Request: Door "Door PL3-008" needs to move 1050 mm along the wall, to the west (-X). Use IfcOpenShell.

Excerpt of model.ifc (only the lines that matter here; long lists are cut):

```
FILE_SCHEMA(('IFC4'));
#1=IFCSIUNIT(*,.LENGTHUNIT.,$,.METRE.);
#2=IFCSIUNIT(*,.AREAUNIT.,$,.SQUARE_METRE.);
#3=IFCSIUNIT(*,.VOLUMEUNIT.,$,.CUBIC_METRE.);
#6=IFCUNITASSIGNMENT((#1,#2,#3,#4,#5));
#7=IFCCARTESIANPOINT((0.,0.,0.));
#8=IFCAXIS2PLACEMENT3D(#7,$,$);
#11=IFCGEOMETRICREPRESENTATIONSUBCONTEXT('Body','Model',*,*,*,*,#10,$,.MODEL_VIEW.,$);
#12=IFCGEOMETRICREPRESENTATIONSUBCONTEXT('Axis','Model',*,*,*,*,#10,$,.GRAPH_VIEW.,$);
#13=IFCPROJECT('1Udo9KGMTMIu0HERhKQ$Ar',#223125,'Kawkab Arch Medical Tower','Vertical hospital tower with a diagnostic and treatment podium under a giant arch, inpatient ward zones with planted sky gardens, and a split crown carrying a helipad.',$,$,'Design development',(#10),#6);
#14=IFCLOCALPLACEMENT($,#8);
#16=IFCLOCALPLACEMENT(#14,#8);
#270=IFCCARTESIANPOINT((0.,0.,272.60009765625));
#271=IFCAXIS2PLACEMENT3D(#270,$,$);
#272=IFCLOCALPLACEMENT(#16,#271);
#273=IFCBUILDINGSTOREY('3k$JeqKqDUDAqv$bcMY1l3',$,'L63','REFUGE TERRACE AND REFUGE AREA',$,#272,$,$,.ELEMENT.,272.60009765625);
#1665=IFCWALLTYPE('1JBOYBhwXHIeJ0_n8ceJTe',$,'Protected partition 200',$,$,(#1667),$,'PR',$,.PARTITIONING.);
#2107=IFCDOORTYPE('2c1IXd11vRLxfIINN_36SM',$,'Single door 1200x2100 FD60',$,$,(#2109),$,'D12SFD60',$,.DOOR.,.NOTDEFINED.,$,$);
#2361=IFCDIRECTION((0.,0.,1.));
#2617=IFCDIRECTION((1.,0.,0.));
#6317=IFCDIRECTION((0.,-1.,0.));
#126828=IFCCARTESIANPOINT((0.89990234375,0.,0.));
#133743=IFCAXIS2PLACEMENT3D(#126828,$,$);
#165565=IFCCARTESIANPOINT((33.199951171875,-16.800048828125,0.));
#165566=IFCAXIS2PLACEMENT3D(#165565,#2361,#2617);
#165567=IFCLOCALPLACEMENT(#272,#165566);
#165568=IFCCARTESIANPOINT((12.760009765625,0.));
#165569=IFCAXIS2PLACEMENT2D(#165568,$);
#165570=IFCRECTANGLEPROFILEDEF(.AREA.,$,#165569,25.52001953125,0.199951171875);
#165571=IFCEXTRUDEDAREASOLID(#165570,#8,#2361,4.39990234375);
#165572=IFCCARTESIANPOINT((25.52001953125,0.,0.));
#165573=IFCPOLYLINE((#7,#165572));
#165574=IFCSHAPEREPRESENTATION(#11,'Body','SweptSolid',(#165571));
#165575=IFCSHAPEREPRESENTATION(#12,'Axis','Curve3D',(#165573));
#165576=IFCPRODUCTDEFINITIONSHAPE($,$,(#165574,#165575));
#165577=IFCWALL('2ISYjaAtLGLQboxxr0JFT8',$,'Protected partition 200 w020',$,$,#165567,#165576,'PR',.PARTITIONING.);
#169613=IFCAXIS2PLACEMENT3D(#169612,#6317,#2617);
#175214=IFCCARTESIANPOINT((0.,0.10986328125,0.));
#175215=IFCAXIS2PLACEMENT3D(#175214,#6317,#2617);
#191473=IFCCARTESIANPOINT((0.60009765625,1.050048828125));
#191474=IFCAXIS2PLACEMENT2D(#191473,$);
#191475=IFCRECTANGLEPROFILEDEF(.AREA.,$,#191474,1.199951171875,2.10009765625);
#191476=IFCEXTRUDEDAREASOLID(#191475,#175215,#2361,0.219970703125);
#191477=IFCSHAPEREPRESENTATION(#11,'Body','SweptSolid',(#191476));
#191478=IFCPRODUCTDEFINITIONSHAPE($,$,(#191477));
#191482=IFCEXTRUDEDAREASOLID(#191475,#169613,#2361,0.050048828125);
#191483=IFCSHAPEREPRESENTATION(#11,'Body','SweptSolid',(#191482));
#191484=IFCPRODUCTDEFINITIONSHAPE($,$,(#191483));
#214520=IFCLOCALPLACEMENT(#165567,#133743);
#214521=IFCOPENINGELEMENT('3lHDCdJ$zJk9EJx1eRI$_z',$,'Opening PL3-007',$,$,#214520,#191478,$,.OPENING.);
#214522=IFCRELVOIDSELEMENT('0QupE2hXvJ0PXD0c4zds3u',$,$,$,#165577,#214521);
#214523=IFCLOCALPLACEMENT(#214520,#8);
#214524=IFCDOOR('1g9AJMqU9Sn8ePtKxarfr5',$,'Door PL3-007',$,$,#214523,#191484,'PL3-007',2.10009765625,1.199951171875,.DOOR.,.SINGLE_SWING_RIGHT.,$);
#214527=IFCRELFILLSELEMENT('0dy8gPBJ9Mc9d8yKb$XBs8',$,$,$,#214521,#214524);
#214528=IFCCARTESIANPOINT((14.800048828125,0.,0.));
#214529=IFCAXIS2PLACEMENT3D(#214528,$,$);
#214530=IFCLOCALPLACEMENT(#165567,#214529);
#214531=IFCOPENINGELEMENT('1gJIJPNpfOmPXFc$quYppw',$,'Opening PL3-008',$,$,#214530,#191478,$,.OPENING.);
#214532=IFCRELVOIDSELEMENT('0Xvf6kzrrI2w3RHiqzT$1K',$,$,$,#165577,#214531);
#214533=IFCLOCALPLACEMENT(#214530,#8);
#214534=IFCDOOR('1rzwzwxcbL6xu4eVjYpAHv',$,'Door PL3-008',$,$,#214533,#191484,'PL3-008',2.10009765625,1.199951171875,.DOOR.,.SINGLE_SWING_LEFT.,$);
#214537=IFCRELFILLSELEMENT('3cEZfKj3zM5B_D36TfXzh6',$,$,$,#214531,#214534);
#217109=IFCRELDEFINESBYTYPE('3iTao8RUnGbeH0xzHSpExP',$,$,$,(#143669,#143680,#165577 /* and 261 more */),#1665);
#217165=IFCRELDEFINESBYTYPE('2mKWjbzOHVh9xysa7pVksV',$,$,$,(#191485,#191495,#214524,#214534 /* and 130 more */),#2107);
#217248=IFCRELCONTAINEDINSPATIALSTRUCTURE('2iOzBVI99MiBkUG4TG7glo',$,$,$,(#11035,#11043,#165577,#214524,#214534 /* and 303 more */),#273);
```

```python
import ifcopenshell
import ifcopenshell.api.geometry
import ifcopenshell.util.placement
import ifcopenshell.util.unit

model = ifcopenshell.open("model.ifc")
unit_scale = ifcopenshell.util.unit.calculate_unit_scale(model)

door = model.by_guid("1rzwzwxcbL6xu4eVjYpAHv")
opening = door.FillsVoids[0].RelatingOpeningElement
wall = opening.VoidsElements[0].RelatingBuildingElement

wall_matrix = ifcopenshell.util.placement.get_local_placement(wall.ObjectPlacement)
shift = wall_matrix[:3, 0] * -1.05 / unit_scale
before = ifcopenshell.util.placement.get_local_placement(door.ObjectPlacement)[:3, 3].copy()

# The door is placed relative to its opening, so it follows when the opening moves.
matrix = ifcopenshell.util.placement.get_local_placement(opening.ObjectPlacement)
matrix[:3, 3] += shift
ifcopenshell.api.geometry.edit_object_placement(
    model, product=opening, matrix=matrix, is_si=False, should_transform_children=True
)

after = ifcopenshell.util.placement.get_local_placement(door.ObjectPlacement)[:3, 3]
print("door moved by", (after - before).round(3) + 0.0)

model.write("model_rev.ifc")
```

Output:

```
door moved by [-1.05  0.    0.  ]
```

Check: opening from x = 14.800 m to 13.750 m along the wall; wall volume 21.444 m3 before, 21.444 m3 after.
